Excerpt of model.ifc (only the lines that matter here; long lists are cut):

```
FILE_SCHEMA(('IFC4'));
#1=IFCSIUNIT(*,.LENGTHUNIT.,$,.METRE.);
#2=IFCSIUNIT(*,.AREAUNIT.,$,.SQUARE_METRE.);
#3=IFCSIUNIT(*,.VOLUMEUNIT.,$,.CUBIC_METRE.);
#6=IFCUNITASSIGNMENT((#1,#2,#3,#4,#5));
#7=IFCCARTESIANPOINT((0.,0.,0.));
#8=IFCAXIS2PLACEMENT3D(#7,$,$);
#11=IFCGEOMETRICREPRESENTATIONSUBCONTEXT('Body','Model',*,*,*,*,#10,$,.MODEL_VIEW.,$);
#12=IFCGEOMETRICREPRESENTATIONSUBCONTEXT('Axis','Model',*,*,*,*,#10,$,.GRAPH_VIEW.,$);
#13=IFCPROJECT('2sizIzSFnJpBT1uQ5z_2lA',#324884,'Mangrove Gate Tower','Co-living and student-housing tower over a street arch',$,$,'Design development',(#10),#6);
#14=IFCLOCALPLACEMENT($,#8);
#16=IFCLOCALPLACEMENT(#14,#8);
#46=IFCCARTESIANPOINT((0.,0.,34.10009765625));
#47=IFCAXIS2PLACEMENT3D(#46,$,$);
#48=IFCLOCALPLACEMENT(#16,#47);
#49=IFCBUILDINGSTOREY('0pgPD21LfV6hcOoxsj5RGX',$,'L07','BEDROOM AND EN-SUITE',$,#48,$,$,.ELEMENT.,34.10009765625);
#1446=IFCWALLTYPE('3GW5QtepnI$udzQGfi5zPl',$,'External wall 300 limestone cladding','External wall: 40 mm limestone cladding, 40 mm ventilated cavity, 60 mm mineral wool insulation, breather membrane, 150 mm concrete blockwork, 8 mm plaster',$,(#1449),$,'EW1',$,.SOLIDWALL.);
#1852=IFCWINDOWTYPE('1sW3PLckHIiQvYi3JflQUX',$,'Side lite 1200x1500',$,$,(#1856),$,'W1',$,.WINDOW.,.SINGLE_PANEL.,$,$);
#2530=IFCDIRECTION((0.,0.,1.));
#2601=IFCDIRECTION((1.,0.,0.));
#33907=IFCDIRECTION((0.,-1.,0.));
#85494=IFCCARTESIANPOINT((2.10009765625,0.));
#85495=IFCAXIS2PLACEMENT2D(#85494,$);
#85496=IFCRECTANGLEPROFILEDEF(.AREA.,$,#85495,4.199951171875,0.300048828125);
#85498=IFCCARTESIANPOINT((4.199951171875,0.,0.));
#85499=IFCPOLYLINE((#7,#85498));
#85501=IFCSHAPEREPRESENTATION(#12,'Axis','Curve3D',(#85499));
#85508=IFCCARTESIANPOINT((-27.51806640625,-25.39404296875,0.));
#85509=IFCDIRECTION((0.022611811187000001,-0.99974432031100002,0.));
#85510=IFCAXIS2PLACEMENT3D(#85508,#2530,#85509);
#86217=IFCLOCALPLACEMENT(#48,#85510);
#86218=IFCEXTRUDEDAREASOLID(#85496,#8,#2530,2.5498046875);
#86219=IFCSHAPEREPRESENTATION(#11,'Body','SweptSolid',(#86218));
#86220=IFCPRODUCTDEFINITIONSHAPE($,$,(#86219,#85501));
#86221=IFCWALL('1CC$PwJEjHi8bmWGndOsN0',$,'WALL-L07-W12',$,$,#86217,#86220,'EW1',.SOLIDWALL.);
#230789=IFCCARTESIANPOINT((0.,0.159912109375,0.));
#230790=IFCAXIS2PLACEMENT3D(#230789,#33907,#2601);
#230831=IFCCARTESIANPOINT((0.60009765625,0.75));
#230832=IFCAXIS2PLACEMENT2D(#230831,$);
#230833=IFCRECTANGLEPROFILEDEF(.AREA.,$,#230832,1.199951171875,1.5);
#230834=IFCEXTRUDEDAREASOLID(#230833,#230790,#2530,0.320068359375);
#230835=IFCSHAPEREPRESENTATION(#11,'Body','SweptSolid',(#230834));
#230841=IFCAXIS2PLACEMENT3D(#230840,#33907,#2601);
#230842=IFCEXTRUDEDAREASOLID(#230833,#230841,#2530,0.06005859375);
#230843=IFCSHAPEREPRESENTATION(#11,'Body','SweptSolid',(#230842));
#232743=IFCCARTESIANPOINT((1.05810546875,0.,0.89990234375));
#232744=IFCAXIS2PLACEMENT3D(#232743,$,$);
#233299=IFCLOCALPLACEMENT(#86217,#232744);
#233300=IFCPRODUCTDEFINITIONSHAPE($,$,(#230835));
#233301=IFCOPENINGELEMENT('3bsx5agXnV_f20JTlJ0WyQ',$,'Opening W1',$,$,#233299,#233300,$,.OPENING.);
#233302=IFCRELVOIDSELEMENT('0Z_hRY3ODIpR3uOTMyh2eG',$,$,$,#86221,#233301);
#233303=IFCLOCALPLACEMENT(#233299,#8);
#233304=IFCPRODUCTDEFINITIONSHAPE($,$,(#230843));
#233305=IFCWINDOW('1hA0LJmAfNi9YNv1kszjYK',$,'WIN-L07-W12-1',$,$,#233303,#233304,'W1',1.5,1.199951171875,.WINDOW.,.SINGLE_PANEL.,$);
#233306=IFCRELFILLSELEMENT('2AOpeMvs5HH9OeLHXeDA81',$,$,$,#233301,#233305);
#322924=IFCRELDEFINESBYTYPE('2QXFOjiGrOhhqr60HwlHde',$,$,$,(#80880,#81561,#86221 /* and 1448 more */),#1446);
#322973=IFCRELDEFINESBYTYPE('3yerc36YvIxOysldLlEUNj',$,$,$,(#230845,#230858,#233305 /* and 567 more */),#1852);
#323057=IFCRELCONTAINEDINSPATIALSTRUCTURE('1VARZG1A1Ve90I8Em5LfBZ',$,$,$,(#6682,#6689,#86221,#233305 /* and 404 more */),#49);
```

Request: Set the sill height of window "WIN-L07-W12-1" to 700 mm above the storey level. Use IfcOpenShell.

```python
import numpy as np
import ifcopenshell
import ifcopenshell.api.geometry
import ifcopenshell.geom
import ifcopenshell.util.element
import ifcopenshell.util.placement
import ifcopenshell.util.shape
import ifcopenshell.util.unit

model = ifcopenshell.open("model.ifc")
unit_scale = ifcopenshell.util.unit.calculate_unit_scale(model)

window = model.by_guid("1hA0LJmAfNi9YNv1kszjYK")
opening = window.FillsVoids[0].RelatingOpeningElement
storey = ifcopenshell.util.element.get_container(window, ifc_class="IfcBuildingStorey")
level = ifcopenshell.util.placement.get_local_placement(storey.ObjectPlacement)[2, 3]

# The opening's origin need not be at the sill, so measure its lowest point.
shape = ifcopenshell.geom.create_shape(ifcopenshell.geom.settings(), opening)
bottom = ifcopenshell.util.shape.get_shape_bottom_elevation(shape, shape.geometry) / unit_scale
dz = level + 0.7 - bottom

shift = np.array([0.0, 0.0, dz])
# The window is placed relative to its opening, so it follows when the opening moves.
matrix = ifcopenshell.util.placement.get_local_placement(opening.ObjectPlacement)
matrix[:3, 3] += shift
ifcopenshell.api.geometry.edit_object_placement(
    model, product=opening, matrix=matrix, is_si=False, should_transform_children=True
)

print(f"moved by {dz * unit_scale:+.3f} m")

model.write("model_rev.ifc")
```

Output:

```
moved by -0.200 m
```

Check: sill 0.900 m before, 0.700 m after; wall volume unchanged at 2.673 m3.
